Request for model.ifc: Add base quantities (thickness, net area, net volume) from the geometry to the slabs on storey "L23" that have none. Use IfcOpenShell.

First a look at what the model holds.

```python
import ifcopenshell
import ifcopenshell.util.element
import ifcopenshell.util.unit

model = ifcopenshell.open("model.ifc")
print(model.schema)
for unit_type in ("LENGTHUNIT", "AREAUNIT", "VOLUMEUNIT"):
    print(unit_type, ifcopenshell.util.unit.calculate_unit_scale(model, unit_type))
storey = next(s for s in model.by_type("IfcBuildingStorey") if s.Name == "L23")
slabs = [e for e in ifcopenshell.util.element.get_decomposition(storey) if e.is_a("IfcSlab")]
for e in sorted(slabs, key=lambda e: e.id()):
    print(e.id(), e.is_a(), e.Name, list(ifcopenshell.util.element.get_psets(e, qtos_only=True)), sep=" | ")
```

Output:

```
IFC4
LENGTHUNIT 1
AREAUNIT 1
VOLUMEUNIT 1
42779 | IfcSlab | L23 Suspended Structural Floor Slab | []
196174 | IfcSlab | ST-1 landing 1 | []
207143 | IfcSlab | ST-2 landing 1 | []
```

```python
import ifcopenshell
import ifcopenshell.api.pset
import ifcopenshell.geom
import ifcopenshell.util.element
import ifcopenshell.util.shape
import ifcopenshell.util.unit

model = ifcopenshell.open("model.ifc")
unit_scale = ifcopenshell.util.unit.calculate_unit_scale(model)
area_scale = ifcopenshell.util.unit.calculate_unit_scale(model, "AREAUNIT")
volume_scale = ifcopenshell.util.unit.calculate_unit_scale(model, "VOLUMEUNIT")
settings = ifcopenshell.geom.settings()

storey = next(s for s in model.by_type("IfcBuildingStorey") if s.Name == "L23")
slabs = [e for e in ifcopenshell.util.element.get_decomposition(storey) if e.is_a("IfcSlab")]

for e in sorted(slabs, key=lambda e: e.id()):
    if ifcopenshell.util.element.get_psets(e, qtos_only=True, should_inherit=False):
        continue
    # Geometry comes back in metres, in the element's own axes.
    shape = ifcopenshell.geom.create_shape(settings, e)
    values = {
        "Width": ifcopenshell.util.shape.get_z(shape.geometry) / unit_scale,
        "NetArea": ifcopenshell.util.shape.get_footprint_area(shape.geometry) / area_scale,
        "NetVolume": ifcopenshell.util.shape.get_volume(shape.geometry) / volume_scale,
    }
    qto = ifcopenshell.api.pset.add_qto(model, product=e, name="Qto_SlabBaseQuantities")
    ifcopenshell.api.pset.edit_qto(model, qto=qto, properties=values)
    print(e.id(), {k: round(v, 3) for k, v in values.items()})

model.write("model_updated.ifc")
```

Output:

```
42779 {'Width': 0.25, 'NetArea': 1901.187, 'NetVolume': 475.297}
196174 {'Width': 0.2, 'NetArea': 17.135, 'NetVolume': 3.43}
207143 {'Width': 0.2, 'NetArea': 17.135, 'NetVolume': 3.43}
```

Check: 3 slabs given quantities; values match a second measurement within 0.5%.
